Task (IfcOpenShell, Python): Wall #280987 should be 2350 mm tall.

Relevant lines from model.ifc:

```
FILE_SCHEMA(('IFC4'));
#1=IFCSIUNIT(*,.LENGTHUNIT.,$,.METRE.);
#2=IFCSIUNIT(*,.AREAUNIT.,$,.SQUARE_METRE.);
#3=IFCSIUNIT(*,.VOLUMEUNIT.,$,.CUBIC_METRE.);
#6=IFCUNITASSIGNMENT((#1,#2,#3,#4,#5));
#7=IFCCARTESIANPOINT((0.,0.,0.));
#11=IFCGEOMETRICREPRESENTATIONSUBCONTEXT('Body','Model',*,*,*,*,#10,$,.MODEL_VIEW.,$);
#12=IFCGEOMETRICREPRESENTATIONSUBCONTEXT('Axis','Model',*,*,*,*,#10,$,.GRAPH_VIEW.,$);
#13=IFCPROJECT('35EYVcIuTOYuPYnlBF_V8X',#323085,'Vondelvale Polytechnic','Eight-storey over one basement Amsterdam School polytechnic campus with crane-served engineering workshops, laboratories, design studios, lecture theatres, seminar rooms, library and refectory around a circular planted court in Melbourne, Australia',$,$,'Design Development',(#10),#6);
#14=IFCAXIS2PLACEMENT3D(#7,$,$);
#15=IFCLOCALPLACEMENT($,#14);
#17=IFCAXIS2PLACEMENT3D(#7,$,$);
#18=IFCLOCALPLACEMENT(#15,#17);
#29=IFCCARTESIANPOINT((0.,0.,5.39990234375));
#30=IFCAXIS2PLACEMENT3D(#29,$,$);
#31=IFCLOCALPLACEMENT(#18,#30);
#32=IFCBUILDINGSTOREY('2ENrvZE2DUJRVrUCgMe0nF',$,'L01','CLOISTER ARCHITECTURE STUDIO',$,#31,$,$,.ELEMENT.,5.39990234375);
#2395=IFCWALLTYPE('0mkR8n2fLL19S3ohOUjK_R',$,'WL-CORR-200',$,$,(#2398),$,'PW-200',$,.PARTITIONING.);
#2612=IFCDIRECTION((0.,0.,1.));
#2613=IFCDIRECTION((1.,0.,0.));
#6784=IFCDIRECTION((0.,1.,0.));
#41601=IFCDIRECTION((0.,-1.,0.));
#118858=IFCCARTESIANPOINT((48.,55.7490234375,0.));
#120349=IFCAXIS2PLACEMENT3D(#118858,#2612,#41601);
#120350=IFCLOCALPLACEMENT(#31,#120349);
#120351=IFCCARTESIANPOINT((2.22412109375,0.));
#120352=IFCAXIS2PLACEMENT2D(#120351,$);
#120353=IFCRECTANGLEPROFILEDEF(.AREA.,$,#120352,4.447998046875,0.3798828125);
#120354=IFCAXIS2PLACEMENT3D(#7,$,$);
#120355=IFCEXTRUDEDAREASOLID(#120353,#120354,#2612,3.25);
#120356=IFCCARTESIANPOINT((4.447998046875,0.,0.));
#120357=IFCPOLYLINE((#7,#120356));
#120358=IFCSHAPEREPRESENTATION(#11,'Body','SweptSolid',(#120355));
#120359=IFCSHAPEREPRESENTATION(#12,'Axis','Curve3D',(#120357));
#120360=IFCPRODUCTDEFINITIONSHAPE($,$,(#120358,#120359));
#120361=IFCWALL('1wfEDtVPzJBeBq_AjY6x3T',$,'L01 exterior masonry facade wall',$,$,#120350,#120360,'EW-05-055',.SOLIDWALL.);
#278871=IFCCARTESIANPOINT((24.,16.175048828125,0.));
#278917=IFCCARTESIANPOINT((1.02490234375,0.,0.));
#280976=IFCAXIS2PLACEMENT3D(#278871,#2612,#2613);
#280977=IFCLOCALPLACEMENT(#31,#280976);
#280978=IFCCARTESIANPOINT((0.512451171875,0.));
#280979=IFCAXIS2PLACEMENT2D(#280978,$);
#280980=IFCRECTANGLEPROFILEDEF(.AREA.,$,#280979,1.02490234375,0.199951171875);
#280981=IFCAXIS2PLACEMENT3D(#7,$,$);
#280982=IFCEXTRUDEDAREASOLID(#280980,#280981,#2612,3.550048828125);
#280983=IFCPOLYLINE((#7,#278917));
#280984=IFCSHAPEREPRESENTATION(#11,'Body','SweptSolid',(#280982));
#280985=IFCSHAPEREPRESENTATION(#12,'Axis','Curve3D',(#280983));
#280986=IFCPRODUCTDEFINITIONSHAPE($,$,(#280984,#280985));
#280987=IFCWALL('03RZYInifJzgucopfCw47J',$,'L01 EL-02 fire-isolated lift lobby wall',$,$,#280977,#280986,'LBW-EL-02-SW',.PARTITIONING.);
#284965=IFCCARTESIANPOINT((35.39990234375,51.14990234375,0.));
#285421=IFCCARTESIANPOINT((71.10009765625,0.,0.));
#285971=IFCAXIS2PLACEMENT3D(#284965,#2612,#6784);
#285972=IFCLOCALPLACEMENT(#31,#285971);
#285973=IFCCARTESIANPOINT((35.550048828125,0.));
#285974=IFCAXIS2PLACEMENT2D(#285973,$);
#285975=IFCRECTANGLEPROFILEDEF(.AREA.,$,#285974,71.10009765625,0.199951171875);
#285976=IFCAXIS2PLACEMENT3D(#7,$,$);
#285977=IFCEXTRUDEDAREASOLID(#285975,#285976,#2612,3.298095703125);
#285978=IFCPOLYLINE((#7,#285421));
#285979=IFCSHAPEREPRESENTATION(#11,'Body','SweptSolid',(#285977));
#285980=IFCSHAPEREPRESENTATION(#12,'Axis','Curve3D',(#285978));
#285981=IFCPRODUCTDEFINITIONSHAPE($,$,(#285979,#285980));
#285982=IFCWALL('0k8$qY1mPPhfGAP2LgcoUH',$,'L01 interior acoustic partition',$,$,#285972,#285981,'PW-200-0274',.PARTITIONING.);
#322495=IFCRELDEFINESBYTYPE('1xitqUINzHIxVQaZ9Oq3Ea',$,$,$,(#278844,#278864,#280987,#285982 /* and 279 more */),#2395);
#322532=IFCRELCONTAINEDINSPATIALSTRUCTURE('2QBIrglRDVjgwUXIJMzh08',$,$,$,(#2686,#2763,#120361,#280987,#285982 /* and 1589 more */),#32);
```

```python
import ifcopenshell
import ifcopenshell.geom
import ifcopenshell.util.representation
import ifcopenshell.util.shape

model = ifcopenshell.open("model.ifc")
settings = ifcopenshell.geom.settings()


def volume(element):
    """Net volume in cubic metres, openings subtracted."""
    shape = ifcopenshell.geom.create_shape(settings, element)
    return ifcopenshell.util.shape.get_volume(shape.geometry)


wall = model.by_id(280987)
before = volume(wall)

body = ifcopenshell.util.representation.get_representation(wall, "Model", "Body")
solid = body.Items[0]
old_height = solid.Depth
solid.Depth = 2.35
after = volume(wall)

print(f"height {old_height:g} -> {solid.Depth:g}, volume {before:.3f} -> {after:.3f} m3")

model.write("model_updated.ifc")
```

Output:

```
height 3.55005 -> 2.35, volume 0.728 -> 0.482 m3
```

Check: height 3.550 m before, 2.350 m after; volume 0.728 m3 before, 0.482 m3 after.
